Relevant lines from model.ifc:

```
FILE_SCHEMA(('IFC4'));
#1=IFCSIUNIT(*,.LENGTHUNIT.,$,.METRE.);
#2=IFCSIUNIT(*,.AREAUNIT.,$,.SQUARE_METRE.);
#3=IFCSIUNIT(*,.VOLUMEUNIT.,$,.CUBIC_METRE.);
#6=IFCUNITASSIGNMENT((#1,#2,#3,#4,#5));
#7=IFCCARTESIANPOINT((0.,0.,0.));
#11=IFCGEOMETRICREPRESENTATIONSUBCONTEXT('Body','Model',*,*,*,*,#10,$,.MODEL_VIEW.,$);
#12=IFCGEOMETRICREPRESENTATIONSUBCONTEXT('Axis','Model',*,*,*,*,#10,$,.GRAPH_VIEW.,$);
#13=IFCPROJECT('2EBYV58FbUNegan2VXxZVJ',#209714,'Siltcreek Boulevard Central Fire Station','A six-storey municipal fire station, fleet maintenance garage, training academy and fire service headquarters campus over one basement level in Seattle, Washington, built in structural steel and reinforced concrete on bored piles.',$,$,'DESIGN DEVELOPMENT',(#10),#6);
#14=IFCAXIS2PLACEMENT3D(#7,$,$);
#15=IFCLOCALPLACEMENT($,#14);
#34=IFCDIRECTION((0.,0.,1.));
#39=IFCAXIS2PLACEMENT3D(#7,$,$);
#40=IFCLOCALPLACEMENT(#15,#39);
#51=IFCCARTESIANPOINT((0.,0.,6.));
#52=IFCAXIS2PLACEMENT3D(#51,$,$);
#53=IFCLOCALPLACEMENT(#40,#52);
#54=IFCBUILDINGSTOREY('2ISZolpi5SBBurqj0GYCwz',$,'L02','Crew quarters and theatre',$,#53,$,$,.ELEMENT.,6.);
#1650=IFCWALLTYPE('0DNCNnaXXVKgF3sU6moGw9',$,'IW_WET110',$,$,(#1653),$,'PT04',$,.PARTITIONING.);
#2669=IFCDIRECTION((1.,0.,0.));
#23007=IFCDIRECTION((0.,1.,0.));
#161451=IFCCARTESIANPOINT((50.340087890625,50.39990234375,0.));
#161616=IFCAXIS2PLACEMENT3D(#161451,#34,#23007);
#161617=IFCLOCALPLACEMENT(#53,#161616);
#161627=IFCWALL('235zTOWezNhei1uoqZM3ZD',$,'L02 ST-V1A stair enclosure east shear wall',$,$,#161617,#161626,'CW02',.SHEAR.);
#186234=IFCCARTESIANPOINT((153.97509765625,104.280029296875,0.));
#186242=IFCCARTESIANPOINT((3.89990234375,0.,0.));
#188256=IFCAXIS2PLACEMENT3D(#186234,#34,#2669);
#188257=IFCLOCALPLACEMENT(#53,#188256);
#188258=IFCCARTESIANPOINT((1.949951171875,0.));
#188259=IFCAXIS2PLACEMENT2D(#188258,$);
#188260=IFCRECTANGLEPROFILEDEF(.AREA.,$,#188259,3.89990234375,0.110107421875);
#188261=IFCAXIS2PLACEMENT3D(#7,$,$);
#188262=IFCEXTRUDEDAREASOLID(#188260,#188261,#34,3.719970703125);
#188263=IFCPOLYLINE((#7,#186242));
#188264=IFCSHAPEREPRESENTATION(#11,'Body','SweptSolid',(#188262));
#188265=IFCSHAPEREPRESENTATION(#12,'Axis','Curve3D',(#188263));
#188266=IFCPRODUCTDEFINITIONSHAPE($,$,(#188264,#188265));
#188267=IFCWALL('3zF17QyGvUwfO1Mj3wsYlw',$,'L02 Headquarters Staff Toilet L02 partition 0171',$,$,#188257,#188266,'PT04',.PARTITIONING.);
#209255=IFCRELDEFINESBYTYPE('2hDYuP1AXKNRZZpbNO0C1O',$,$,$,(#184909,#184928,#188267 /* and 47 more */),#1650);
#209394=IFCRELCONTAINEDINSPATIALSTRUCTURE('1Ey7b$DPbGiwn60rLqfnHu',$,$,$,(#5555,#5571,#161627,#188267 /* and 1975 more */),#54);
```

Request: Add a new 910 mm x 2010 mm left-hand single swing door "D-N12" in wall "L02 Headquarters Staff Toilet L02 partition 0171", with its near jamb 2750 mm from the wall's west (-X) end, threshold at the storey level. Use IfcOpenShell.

```python
import numpy as np
import ifcopenshell
import ifcopenshell.api.feature
import ifcopenshell.api.geometry
import ifcopenshell.api.root
import ifcopenshell.api.spatial
import ifcopenshell.geom
import ifcopenshell.util.element
import ifcopenshell.util.placement
import ifcopenshell.util.representation
import ifcopenshell.util.shape
import ifcopenshell.util.unit

model = ifcopenshell.open("model.ifc")
unit_scale = ifcopenshell.util.unit.calculate_unit_scale(model)
settings = ifcopenshell.geom.settings()


def volume(element):
    """Net volume in cubic metres, openings subtracted."""
    shape = ifcopenshell.geom.create_shape(settings, element)
    return ifcopenshell.util.shape.get_volume(shape.geometry)


wall = model.by_guid("3zF17QyGvUwfO1Mj3wsYlw")
storey = ifcopenshell.util.element.get_container(wall, ifc_class="IfcBuildingStorey")
context = ifcopenshell.util.representation.get_context(model, "Model", "Body", "MODEL_VIEW")
before = volume(wall)

width, height, from_end, sill = 0.91, 2.01, 2.75, 0.0  # metres

# The wall runs along its own X axis, and the end named is its -X end.
wall_shape = ifcopenshell.geom.create_shape(settings, wall)
x, y, z = ifcopenshell.util.shape.get_vertices(wall_shape.geometry).T
start = x.min() + from_end
face, thickness = float(y.min()), float(y.max() - y.min())
wall_matrix = ifcopenshell.util.placement.get_local_placement(wall.ObjectPlacement)
level = ifcopenshell.util.placement.get_local_placement(storey.ObjectPlacement)[2, 3]


def in_wall(x, y):
    """Placement at x, y metres in the wall's axes, at sill height."""
    matrix = wall_matrix.copy()
    matrix[:, 3] = wall_matrix @ np.array([x / unit_scale, y / unit_scale, 0.0, 1.0])
    matrix[2, 3] = level + sill / unit_scale
    return matrix


# Opening: a box that overshoots both wall faces by 50 mm.
opening = ifcopenshell.api.root.create_entity(model, ifc_class="IfcOpeningElement", predefined_type="OPENING")
box = ifcopenshell.api.geometry.add_wall_representation(
    model, context=context, length=width, height=height, thickness=thickness + 0.1
)
ifcopenshell.api.geometry.assign_representation(model, product=opening, representation=box)
ifcopenshell.api.geometry.edit_object_placement(model, product=opening, matrix=in_wall(start, face - 0.05), is_si=False)
ifcopenshell.api.feature.add_feature(model, feature=opening, element=wall)

door = ifcopenshell.api.root.create_entity(model, ifc_class="IfcDoor", name="D-N12", predefined_type="DOOR")
door.OverallWidth, door.OverallHeight = width / unit_scale, height / unit_scale
door.OperationType = "SINGLE_SWING_LEFT"
body = ifcopenshell.api.geometry.add_door_representation(
    model,
    context=context,
    overall_width=door.OverallWidth,
    overall_height=door.OverallHeight,
    operation_type="SINGLE_SWING_LEFT",
    lining_properties={"LiningDepth": thickness / unit_scale, "ThresholdDepth": thickness / unit_scale},
)
ifcopenshell.api.geometry.assign_representation(model, product=door, representation=body)
ifcopenshell.api.spatial.assign_container(model, products=[door], relating_structure=storey)
ifcopenshell.api.feature.add_filling(model, opening=opening, element=door)

# The lining spans the wall, so the door starts at the wall face.
ifcopenshell.api.geometry.edit_object_placement(model, product=door, matrix=in_wall(start, face), is_si=False)

after = volume(wall)

print(f"wall volume {before:.3f} -> {after:.3f} m3")

model.write("model_rev.ifc")
```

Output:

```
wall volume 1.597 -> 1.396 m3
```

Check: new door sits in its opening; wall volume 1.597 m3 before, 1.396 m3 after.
